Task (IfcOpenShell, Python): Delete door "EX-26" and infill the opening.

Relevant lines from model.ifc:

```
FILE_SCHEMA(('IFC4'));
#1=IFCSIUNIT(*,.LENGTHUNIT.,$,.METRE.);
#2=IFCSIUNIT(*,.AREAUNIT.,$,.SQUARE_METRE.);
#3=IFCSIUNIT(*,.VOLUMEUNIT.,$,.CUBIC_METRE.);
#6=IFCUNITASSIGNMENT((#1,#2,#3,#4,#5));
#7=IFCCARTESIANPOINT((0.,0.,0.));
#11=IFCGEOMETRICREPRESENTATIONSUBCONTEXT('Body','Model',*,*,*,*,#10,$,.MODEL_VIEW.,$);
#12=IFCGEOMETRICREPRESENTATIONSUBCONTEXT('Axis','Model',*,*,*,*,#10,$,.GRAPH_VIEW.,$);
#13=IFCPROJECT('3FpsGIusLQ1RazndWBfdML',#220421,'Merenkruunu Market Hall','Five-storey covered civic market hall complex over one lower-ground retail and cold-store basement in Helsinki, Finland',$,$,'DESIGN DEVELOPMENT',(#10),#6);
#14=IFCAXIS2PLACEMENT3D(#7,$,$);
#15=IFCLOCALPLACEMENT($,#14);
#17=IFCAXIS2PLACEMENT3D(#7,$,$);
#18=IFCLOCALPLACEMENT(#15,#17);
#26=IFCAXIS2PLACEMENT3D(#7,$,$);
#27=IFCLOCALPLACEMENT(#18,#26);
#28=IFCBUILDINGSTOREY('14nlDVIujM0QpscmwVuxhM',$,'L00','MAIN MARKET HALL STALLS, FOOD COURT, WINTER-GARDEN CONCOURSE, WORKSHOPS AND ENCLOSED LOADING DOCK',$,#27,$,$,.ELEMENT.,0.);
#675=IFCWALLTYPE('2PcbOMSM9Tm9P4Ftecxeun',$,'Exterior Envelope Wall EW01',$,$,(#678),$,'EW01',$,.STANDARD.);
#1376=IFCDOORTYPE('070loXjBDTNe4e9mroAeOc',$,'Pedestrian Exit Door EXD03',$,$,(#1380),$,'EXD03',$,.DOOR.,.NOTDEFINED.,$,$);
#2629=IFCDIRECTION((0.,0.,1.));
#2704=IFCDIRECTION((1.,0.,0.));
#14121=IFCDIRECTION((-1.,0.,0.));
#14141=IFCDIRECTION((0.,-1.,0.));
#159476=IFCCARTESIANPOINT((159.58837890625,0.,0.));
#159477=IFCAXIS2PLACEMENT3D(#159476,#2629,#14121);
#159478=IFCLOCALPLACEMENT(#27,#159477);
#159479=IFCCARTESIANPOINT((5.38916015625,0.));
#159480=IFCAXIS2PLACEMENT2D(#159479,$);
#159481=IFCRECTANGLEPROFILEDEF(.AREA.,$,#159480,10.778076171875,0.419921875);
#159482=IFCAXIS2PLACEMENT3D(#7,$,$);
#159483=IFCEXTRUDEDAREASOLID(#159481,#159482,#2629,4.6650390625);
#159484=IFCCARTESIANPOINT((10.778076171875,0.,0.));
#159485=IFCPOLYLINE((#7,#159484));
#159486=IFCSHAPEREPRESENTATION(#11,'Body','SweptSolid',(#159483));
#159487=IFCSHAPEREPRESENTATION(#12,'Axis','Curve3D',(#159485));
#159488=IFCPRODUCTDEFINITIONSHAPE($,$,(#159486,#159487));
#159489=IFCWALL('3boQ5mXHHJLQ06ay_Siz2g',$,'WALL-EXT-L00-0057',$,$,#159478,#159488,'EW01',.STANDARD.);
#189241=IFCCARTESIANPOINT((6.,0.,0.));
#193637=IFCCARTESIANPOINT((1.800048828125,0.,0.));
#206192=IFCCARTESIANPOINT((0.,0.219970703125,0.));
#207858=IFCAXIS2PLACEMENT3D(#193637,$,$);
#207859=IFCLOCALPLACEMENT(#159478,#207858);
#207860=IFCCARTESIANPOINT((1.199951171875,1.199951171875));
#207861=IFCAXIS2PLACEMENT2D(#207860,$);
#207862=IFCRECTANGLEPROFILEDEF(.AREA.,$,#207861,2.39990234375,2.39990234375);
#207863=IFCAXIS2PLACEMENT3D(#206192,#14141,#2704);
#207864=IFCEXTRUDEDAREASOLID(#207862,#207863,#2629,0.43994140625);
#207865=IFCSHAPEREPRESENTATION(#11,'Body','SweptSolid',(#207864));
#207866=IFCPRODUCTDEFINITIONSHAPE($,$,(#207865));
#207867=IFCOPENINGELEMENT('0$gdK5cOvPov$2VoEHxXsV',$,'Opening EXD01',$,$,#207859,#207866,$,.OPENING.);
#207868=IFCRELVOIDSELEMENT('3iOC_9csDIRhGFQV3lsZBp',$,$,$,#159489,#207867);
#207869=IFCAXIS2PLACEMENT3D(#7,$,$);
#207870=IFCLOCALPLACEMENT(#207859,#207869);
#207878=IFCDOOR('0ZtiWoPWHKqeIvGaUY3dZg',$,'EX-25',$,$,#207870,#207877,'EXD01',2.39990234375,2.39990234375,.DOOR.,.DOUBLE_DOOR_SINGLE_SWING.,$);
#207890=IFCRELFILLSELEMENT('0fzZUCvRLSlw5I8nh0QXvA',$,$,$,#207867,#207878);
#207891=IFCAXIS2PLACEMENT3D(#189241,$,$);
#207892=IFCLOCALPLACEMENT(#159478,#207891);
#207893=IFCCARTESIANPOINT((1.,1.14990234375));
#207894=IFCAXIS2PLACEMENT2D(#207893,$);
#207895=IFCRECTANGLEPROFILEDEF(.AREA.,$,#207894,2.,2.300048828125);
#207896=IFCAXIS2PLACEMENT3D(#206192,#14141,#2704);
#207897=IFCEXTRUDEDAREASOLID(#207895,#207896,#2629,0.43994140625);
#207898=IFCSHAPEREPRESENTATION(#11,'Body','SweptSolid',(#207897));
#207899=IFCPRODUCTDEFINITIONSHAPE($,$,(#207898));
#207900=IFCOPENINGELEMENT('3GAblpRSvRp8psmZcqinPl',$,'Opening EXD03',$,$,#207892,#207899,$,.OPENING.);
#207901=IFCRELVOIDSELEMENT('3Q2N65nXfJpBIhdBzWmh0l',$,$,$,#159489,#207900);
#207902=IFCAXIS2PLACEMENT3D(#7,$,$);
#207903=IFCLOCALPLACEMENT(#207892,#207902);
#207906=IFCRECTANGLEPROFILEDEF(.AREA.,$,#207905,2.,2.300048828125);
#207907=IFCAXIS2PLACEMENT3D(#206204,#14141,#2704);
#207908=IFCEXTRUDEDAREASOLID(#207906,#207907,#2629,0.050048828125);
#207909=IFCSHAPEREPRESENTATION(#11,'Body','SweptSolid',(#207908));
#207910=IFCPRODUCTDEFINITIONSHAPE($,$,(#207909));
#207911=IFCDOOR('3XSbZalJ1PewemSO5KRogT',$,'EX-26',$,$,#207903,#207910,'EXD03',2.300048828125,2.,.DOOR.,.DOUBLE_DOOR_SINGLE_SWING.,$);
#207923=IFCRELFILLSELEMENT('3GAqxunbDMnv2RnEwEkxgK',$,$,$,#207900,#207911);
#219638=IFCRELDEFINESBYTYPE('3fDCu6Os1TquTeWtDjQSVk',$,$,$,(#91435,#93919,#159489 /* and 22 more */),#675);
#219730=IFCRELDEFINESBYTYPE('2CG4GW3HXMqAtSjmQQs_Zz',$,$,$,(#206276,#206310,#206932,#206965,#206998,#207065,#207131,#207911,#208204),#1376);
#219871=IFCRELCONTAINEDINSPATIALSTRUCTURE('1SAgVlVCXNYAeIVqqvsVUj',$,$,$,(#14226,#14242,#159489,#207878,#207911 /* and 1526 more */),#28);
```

```python
import ifcopenshell
import ifcopenshell.api.feature
import ifcopenshell.api.root
import ifcopenshell.geom
import ifcopenshell.util.shape

model = ifcopenshell.open("model.ifc")
settings = ifcopenshell.geom.settings()


def volume(element):
    """Net volume in cubic metres, openings subtracted."""
    shape = ifcopenshell.geom.create_shape(settings, element)
    return ifcopenshell.util.shape.get_volume(shape.geometry)


door = model.by_id(207911)
opening = door.FillsVoids[0].RelatingOpeningElement
wall = opening.VoidsElements[0].RelatingBuildingElement
before = volume(wall)

ifcopenshell.api.root.remove_product(model, product=door)
ifcopenshell.api.feature.remove_feature(model, feature=opening)

after = volume(wall)

print(f"wall volume {before:.3f} -> {after:.3f} m3")

model.write("model_rev.ifc")
```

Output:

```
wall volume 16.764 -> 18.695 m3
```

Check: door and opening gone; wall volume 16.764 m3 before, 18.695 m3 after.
